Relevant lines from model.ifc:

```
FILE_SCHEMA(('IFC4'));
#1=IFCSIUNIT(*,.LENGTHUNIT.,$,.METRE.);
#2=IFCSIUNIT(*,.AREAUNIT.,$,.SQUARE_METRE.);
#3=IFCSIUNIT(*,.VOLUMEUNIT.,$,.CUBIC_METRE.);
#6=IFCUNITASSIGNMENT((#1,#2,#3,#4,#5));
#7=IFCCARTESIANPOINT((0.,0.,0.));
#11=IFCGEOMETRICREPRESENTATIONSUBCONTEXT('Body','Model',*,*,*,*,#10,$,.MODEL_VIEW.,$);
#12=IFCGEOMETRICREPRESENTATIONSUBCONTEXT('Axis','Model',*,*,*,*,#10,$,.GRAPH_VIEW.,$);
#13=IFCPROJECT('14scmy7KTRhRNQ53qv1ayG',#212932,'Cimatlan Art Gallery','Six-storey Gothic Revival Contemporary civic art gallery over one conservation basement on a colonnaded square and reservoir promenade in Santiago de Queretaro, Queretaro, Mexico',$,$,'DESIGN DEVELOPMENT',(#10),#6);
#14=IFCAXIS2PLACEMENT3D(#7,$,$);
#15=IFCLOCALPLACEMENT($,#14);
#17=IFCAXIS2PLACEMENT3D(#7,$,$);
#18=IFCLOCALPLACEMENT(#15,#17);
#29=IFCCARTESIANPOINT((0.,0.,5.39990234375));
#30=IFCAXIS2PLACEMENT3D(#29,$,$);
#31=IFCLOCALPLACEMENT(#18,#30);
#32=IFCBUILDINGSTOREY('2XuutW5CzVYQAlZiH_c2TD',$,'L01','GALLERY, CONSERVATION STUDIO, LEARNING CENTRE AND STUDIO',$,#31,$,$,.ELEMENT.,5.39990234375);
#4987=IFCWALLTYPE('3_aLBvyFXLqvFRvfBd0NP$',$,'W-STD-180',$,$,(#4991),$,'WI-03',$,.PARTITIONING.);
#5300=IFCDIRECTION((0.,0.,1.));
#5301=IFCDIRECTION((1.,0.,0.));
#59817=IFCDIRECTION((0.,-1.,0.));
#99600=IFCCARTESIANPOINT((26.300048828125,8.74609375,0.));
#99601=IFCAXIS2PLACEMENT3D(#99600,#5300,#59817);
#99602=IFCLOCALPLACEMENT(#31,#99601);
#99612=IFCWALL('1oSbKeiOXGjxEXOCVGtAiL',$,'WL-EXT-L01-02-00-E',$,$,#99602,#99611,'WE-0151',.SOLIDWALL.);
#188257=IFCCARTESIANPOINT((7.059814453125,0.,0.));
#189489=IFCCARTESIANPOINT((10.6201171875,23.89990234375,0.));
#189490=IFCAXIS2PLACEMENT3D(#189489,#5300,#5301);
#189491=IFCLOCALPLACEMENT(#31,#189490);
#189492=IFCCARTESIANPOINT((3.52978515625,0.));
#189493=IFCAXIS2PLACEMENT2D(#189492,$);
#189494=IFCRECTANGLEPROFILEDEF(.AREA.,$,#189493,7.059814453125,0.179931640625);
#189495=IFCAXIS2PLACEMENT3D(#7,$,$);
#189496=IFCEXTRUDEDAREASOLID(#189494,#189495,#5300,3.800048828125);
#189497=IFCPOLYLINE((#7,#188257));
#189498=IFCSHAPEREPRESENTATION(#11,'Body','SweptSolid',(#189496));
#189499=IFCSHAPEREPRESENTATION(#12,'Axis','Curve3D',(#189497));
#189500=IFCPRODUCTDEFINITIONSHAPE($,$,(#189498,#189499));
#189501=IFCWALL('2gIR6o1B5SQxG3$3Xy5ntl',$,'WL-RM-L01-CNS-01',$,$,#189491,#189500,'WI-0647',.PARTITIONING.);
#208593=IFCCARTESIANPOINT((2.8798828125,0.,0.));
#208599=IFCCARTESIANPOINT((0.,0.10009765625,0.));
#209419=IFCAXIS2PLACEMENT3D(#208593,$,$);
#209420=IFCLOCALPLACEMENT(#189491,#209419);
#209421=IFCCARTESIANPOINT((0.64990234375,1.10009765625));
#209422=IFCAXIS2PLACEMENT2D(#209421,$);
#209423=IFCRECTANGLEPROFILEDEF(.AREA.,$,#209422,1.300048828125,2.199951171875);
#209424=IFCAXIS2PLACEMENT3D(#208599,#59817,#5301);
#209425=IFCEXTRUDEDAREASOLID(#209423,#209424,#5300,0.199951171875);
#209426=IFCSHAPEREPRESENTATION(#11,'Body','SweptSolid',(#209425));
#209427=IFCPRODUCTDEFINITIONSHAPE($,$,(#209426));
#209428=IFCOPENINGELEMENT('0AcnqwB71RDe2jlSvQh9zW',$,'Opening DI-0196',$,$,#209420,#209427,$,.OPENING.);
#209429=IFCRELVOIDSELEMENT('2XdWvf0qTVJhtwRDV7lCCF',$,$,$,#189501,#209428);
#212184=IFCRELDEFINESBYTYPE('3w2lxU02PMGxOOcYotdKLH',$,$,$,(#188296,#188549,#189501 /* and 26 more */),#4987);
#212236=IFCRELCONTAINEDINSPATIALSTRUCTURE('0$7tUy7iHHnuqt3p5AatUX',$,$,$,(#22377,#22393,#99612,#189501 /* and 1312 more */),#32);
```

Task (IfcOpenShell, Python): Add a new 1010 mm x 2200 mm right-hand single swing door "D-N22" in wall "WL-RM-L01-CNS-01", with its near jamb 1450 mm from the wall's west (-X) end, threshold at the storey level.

```python
import numpy as np
import ifcopenshell
import ifcopenshell.api.feature
import ifcopenshell.api.geometry
import ifcopenshell.api.root
import ifcopenshell.api.spatial
import ifcopenshell.geom
import ifcopenshell.util.element
import ifcopenshell.util.placement
import ifcopenshell.util.representation
import ifcopenshell.util.shape
import ifcopenshell.util.unit

model = ifcopenshell.open("model.ifc")
unit_scale = ifcopenshell.util.unit.calculate_unit_scale(model)
settings = ifcopenshell.geom.settings()


def volume(element):
    """Net volume in cubic metres, openings subtracted."""
    shape = ifcopenshell.geom.create_shape(settings, element)
    return ifcopenshell.util.shape.get_volume(shape.geometry)


wall = model.by_guid("2gIR6o1B5SQxG3$3Xy5ntl")
storey = ifcopenshell.util.element.get_container(wall, ifc_class="IfcBuildingStorey")
context = ifcopenshell.util.representation.get_context(model, "Model", "Body", "MODEL_VIEW")
before = volume(wall)

width, height, from_end, sill = 1.01, 2.2, 1.45, 0.0  # metres

# The wall runs along its own X axis, and the end named is its -X end.
wall_shape = ifcopenshell.geom.create_shape(settings, wall)
x, y, z = ifcopenshell.util.shape.get_vertices(wall_shape.geometry).T
start = x.min() + from_end
face, thickness = float(y.min()), float(y.max() - y.min())
wall_matrix = ifcopenshell.util.placement.get_local_placement(wall.ObjectPlacement)
level = ifcopenshell.util.placement.get_local_placement(storey.ObjectPlacement)[2, 3]


def in_wall(x, y):
    """Placement at x, y metres in the wall's axes, at sill height."""
    matrix = wall_matrix.copy()
    matrix[:, 3] = wall_matrix @ np.array([x / unit_scale, y / unit_scale, 0.0, 1.0])
    matrix[2, 3] = level + sill / unit_scale
    return matrix


# Opening: a box that overshoots both wall faces by 50 mm.
opening = ifcopenshell.api.root.create_entity(model, ifc_class="IfcOpeningElement", predefined_type="OPENING")
box = ifcopenshell.api.geometry.add_wall_representation(
    model, context=context, length=width, height=height, thickness=thickness + 0.1
)
ifcopenshell.api.geometry.assign_representation(model, product=opening, representation=box)
ifcopenshell.api.geometry.edit_object_placement(model, product=opening, matrix=in_wall(start, face - 0.05), is_si=False)
ifcopenshell.api.feature.add_feature(model, feature=opening, element=wall)

door = ifcopenshell.api.root.create_entity(model, ifc_class="IfcDoor", name="D-N22", predefined_type="DOOR")
door.OverallWidth, door.OverallHeight = width / unit_scale, height / unit_scale
door.OperationType = "SINGLE_SWING_RIGHT"
body = ifcopenshell.api.geometry.add_door_representation(
    model,
    context=context,
    overall_width=door.OverallWidth,
    overall_height=door.OverallHeight,
    operation_type="SINGLE_SWING_RIGHT",
    lining_properties={"LiningDepth": thickness / unit_scale, "ThresholdDepth": thickness / unit_scale},
)
ifcopenshell.api.geometry.assign_representation(model, product=door, representation=body)
ifcopenshell.api.spatial.assign_container(model, products=[door], relating_structure=storey)
ifcopenshell.api.feature.add_filling(model, opening=opening, element=door)

# The lining spans the wall, so the door starts at the wall face.
ifcopenshell.api.geometry.edit_object_placement(model, product=door, matrix=in_wall(start, face), is_si=False)

after = volume(wall)

print(f"wall volume {before:.3f} -> {after:.3f} m3")

model.write("model_rev.ifc")
```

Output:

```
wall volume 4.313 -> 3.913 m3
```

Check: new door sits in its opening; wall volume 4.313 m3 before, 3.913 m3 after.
